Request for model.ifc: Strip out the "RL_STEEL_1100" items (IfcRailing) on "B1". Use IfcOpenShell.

First a look at what the model holds.

```python
import ifcopenshell
import ifcopenshell.util.element

model = ifcopenshell.open("model.ifc")
print(model.schema)
storey = next(s for s in model.by_type("IfcBuildingStorey") if s.Name == "B1")
railings = [e for e in ifcopenshell.util.element.get_decomposition(storey) if e.is_a("IfcRailing")]
seen = {}
for e in railings:
    element_type = ifcopenshell.util.element.get_type(e)
    name = element_type.Name if element_type not in (None, e) else None
    seen[name] = seen.get(name, 0) + 1
for name, count in sorted(seen.items(), key=str):
    print(count, "x", name)
```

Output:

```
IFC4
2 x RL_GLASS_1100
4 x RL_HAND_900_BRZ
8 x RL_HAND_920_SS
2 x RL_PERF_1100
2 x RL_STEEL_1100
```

```python
import ifcopenshell
import ifcopenshell.api.root
import ifcopenshell.util.element

model = ifcopenshell.open("model.ifc")

storey = next(s for s in model.by_type("IfcBuildingStorey") if s.Name == "B1")
railings = [e for e in ifcopenshell.util.element.get_decomposition(storey) if e.is_a("IfcRailing")]
targets = [e for e in railings if (t := ifcopenshell.util.element.get_type(e)) not in (None, e) and t.Name == "RL_STEEL_1100"]

for e in targets:
    ifcopenshell.api.root.remove_product(model, product=e)
print(len(targets), "removed")

model.write("model_updated.ifc")
```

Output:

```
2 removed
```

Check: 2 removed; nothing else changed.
